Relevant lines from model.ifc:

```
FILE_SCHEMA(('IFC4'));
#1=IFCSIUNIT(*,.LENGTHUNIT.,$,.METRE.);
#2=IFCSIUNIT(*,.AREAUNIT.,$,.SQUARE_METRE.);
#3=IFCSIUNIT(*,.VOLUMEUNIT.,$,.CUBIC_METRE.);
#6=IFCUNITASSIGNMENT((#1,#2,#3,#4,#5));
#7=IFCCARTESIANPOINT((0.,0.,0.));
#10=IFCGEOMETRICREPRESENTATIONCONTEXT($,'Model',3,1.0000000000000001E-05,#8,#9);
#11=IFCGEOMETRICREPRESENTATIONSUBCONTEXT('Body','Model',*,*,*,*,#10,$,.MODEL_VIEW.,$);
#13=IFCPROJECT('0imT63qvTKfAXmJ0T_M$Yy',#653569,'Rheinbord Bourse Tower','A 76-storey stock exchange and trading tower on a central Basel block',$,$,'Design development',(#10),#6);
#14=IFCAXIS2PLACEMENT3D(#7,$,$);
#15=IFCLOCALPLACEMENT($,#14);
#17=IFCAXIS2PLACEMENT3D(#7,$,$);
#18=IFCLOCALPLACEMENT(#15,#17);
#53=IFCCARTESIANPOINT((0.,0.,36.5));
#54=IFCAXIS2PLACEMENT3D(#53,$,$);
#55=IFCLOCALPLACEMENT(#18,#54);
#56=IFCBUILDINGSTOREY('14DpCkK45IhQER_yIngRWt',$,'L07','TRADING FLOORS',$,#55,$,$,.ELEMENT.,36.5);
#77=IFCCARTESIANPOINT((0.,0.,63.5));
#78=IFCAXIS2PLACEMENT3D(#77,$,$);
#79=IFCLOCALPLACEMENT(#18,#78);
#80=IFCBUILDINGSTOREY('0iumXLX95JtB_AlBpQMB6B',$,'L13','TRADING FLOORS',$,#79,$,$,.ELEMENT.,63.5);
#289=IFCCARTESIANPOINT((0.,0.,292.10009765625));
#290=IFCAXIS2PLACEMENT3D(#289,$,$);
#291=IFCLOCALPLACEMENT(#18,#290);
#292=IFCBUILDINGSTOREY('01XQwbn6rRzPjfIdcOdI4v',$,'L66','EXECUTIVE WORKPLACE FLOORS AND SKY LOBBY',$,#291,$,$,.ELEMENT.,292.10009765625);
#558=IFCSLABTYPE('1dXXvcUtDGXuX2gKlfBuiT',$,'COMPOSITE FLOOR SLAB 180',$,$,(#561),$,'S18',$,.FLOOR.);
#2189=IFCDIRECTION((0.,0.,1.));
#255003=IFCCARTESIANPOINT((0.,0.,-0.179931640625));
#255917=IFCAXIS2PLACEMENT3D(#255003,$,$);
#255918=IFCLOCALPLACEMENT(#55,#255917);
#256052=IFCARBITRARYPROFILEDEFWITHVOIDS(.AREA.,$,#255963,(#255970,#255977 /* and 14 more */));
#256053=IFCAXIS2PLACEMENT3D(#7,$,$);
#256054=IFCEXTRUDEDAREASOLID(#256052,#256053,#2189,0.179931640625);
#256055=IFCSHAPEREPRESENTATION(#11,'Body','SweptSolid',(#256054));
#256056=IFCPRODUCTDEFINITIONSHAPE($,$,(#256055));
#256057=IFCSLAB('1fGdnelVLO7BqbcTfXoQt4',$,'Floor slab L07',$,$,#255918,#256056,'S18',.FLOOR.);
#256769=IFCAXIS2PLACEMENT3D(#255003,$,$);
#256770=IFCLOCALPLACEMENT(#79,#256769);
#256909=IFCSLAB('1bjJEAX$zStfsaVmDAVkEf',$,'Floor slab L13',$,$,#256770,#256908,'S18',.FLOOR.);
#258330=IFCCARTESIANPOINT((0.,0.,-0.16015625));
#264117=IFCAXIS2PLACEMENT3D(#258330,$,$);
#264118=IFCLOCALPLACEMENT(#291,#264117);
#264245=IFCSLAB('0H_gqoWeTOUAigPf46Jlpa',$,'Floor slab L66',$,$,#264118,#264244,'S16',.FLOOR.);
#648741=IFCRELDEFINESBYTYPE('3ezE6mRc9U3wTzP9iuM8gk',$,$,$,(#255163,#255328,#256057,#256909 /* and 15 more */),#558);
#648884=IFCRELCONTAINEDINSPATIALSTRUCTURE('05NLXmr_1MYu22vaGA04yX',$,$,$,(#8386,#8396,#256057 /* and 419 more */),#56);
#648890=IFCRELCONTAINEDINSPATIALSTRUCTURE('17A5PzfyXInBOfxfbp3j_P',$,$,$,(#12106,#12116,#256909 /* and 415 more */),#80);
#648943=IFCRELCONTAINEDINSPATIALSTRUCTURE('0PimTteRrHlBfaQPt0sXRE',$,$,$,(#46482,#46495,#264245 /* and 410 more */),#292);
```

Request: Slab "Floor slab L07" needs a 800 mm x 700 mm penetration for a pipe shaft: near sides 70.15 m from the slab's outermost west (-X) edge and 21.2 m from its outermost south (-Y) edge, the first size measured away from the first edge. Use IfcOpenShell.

```python
import numpy as np
import ifcopenshell
import ifcopenshell.api.feature
import ifcopenshell.api.geometry
import ifcopenshell.api.root
import ifcopenshell.geom
import ifcopenshell.util.placement
import ifcopenshell.util.representation
import ifcopenshell.util.shape
import ifcopenshell.util.unit

model = ifcopenshell.open("model.ifc")
unit_scale = ifcopenshell.util.unit.calculate_unit_scale(model)
settings = ifcopenshell.geom.settings()


def volume(element):
    """Net volume in cubic metres, openings subtracted."""
    shape = ifcopenshell.geom.create_shape(settings, element)
    return ifcopenshell.util.shape.get_volume(shape.geometry)


slab = model.by_guid("1fGdnelVLO7BqbcTfXoQt4")
before = volume(slab)

# Extent in the slab's own axes, in metres. The edges named are its -X and -Y sides.
slab_shape = ifcopenshell.geom.create_shape(settings, slab)
vertices = ifcopenshell.util.shape.get_vertices(slab_shape.geometry)
x_min, y_min, bottom = vertices.min(axis=0)
top = vertices[:, 2].max()

opening = ifcopenshell.api.root.create_entity(model, ifc_class="IfcOpeningElement", name="Pipe shaft opening", predefined_type="OPENING")
context = ifcopenshell.util.representation.get_context(model, "Model", "Body", "MODEL_VIEW")
width, depth = 0.8, 0.7
outline = [(0.0, 0.0), (width, 0.0), (width, depth), (0.0, depth), (0.0, 0.0)]
# Overshoot both faces by 50 mm so the cut is clean.
shape = ifcopenshell.api.geometry.add_slab_representation(
    model, context=context, depth=top - bottom + 0.1, polyline=outline
)
ifcopenshell.api.geometry.assign_representation(model, product=opening, representation=shape)

matrix = ifcopenshell.util.placement.get_local_placement(slab.ObjectPlacement)
matrix[:, 3] = matrix @ np.append(np.array([x_min + 70.15, y_min + 21.2, bottom - 0.05]) / unit_scale, 1.0)
ifcopenshell.api.geometry.edit_object_placement(model, product=opening, matrix=matrix, is_si=False)
ifcopenshell.api.feature.add_feature(model, feature=opening, element=slab)

after = volume(slab)

print(f"slab volume {before:.3f} -> {after:.3f} m3")

model.write("model_rev.ifc")
```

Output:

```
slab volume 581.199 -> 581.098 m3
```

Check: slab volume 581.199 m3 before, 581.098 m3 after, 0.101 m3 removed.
